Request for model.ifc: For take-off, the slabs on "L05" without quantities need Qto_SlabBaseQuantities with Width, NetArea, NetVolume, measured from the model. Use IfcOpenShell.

First a look at what the model holds.

```python
import ifcopenshell
import ifcopenshell.util.element
import ifcopenshell.util.unit

model = ifcopenshell.open("model.ifc")
print(model.schema)
for unit_type in ("LENGTHUNIT", "AREAUNIT", "VOLUMEUNIT"):
    print(unit_type, ifcopenshell.util.unit.calculate_unit_scale(model, unit_type))
storey = next(s for s in model.by_type("IfcBuildingStorey") if s.Name == "L05")
slabs = [e for e in ifcopenshell.util.element.get_decomposition(storey) if e.is_a("IfcSlab")]
for e in sorted(slabs, key=lambda e: e.id()):
    print(e.id(), e.is_a(), e.Name, list(ifcopenshell.util.element.get_psets(e, qtos_only=True)), sep=" | ")
```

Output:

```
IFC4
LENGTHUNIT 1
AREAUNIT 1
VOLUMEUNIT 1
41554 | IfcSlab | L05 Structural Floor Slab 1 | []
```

```python
import ifcopenshell
import ifcopenshell.api.pset
import ifcopenshell.geom
import ifcopenshell.util.element
import ifcopenshell.util.shape
import ifcopenshell.util.unit

model = ifcopenshell.open("model.ifc")
unit_scale = ifcopenshell.util.unit.calculate_unit_scale(model)
area_scale = ifcopenshell.util.unit.calculate_unit_scale(model, "AREAUNIT")
volume_scale = ifcopenshell.util.unit.calculate_unit_scale(model, "VOLUMEUNIT")
settings = ifcopenshell.geom.settings()

storey = next(s for s in model.by_type("IfcBuildingStorey") if s.Name == "L05")
slabs = [e for e in ifcopenshell.util.element.get_decomposition(storey) if e.is_a("IfcSlab")]

for e in sorted(slabs, key=lambda e: e.id()):
    if ifcopenshell.util.element.get_psets(e, qtos_only=True, should_inherit=False):
        continue
    # Geometry comes back in metres, in the element's own axes.
    shape = ifcopenshell.geom.create_shape(settings, e)
    values = {
        "Width": ifcopenshell.util.shape.get_z(shape.geometry) / unit_scale,
        "NetArea": ifcopenshell.util.shape.get_footprint_area(shape.geometry) / area_scale,
        "NetVolume": ifcopenshell.util.shape.get_volume(shape.geometry) / volume_scale,
    }
    qto = ifcopenshell.api.pset.add_qto(model, product=e, name="Qto_SlabBaseQuantities")
    ifcopenshell.api.pset.edit_qto(model, qto=qto, properties=values)
    print(e.id(), {k: round(v, 3) for k, v in values.items()})

model.write("model_updated.ifc")
```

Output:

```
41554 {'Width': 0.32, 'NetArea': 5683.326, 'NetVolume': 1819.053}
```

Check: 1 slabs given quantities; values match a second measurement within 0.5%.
